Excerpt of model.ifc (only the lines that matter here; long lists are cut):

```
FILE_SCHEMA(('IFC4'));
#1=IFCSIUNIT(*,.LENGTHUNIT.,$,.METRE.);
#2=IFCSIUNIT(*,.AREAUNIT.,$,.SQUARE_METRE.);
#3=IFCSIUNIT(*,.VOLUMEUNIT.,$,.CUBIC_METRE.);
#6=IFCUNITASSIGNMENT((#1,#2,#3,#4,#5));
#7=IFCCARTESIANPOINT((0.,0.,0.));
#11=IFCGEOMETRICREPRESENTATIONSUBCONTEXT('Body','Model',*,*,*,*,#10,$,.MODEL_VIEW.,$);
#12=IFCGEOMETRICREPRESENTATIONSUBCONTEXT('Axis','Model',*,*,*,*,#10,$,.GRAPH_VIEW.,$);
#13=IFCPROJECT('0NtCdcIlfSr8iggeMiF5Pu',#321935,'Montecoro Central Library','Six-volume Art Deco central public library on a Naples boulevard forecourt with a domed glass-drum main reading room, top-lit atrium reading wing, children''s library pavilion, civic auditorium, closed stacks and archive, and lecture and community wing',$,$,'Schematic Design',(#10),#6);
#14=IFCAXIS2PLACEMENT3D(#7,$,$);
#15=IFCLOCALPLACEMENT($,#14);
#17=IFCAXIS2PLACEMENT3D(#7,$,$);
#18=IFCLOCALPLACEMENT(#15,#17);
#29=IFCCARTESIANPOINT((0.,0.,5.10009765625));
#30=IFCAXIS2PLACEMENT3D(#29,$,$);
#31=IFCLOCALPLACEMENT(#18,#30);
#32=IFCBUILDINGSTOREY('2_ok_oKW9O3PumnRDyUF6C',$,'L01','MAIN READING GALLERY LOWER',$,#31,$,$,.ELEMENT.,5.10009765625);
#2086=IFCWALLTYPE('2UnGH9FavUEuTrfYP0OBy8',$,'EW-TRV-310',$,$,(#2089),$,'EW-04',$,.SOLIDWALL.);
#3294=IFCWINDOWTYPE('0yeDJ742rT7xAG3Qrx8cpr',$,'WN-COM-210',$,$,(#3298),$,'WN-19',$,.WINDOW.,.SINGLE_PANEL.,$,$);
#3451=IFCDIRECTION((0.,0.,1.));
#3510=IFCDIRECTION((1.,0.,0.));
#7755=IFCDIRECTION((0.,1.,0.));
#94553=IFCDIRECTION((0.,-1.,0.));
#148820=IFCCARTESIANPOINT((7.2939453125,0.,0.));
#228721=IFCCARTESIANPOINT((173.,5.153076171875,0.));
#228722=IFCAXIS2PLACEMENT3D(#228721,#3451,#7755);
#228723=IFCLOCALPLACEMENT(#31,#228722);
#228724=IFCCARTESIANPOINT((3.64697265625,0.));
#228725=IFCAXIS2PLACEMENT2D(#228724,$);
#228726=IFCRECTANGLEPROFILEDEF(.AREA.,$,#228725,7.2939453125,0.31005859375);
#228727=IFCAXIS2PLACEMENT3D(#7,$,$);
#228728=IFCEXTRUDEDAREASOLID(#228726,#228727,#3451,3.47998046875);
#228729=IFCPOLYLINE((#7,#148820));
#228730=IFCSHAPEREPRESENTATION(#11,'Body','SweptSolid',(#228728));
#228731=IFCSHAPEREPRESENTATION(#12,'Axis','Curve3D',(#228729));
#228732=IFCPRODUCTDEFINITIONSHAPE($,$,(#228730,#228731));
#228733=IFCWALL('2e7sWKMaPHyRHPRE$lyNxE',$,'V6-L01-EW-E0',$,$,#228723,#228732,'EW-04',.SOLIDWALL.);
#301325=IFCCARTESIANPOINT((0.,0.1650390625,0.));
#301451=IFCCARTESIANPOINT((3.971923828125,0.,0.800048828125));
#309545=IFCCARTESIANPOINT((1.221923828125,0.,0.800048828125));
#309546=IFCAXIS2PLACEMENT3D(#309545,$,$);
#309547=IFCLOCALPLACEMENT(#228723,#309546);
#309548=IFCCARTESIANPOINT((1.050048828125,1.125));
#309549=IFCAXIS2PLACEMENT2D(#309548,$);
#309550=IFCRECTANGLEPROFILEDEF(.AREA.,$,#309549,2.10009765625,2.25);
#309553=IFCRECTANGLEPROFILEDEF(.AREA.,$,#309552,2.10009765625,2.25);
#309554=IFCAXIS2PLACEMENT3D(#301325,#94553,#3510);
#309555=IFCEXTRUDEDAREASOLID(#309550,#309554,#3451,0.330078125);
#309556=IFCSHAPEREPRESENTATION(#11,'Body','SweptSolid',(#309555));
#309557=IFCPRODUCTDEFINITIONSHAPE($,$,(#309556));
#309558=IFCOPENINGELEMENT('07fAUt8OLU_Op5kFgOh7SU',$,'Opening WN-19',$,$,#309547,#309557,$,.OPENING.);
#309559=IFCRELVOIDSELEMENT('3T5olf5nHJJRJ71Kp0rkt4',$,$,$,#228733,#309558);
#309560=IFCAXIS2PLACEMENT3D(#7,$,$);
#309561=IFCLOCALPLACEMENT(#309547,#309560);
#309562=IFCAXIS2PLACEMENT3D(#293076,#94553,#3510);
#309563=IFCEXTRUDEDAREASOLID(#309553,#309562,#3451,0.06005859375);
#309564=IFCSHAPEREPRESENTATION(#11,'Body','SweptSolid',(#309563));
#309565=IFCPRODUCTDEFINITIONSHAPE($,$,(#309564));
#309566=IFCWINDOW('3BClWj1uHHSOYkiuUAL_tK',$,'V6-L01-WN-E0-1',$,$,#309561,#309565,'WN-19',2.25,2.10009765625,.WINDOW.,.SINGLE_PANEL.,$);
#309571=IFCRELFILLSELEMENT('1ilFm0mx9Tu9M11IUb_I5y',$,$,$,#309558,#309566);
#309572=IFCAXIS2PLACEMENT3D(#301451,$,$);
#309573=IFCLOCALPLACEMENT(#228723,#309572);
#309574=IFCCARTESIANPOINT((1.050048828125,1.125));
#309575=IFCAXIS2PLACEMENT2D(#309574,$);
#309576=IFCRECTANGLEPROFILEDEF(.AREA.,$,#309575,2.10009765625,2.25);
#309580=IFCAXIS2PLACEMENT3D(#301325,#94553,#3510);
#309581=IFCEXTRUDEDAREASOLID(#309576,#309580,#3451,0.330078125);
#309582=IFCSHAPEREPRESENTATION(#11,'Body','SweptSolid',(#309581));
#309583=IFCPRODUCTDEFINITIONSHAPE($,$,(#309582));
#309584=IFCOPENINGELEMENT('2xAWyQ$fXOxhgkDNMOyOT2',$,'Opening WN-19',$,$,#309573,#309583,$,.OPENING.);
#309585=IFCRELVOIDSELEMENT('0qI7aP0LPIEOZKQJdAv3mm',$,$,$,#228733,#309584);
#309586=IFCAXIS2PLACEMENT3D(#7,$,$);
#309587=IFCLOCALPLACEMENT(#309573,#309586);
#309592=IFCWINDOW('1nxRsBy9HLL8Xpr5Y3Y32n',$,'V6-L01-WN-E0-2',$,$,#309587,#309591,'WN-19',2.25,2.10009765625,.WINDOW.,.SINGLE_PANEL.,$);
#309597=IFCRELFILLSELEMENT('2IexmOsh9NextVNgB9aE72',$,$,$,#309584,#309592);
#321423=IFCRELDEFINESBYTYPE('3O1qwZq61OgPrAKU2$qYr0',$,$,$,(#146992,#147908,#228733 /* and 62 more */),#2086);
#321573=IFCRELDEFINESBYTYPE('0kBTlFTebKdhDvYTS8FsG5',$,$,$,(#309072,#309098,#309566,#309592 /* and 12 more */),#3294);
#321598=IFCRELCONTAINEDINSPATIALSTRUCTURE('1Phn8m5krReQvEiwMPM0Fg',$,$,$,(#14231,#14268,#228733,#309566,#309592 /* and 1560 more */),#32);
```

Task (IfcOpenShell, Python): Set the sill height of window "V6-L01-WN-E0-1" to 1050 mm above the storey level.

```python
import numpy as np
import ifcopenshell
import ifcopenshell.api.geometry
import ifcopenshell.geom
import ifcopenshell.util.element
import ifcopenshell.util.placement
import ifcopenshell.util.shape
import ifcopenshell.util.unit

model = ifcopenshell.open("model.ifc")
unit_scale = ifcopenshell.util.unit.calculate_unit_scale(model)

window = model.by_guid("3BClWj1uHHSOYkiuUAL_tK")
opening = window.FillsVoids[0].RelatingOpeningElement
storey = ifcopenshell.util.element.get_container(window, ifc_class="IfcBuildingStorey")
level = ifcopenshell.util.placement.get_local_placement(storey.ObjectPlacement)[2, 3]

# The opening's origin need not be at the sill, so measure its lowest point.
shape = ifcopenshell.geom.create_shape(ifcopenshell.geom.settings(), opening)
bottom = ifcopenshell.util.shape.get_shape_bottom_elevation(shape, shape.geometry) / unit_scale
dz = level + 1.05 / unit_scale - bottom

shift = np.array([0.0, 0.0, dz])
# The window is placed relative to its opening, so it follows when the opening moves.
matrix = ifcopenshell.util.placement.get_local_placement(opening.ObjectPlacement)
matrix[:3, 3] += shift
ifcopenshell.api.geometry.edit_object_placement(
    model, product=opening, matrix=matrix, is_si=False, should_transform_children=True
)

print(f"moved by {dz * unit_scale:+.3f} m")

model.write("model_edited.ifc")
```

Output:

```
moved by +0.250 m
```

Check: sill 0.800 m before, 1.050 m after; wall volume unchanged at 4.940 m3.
